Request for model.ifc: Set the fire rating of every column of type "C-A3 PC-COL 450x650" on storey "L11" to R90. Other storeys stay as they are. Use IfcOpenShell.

First a look at what the model holds.

```python
import ifcopenshell
import ifcopenshell.util.element

model = ifcopenshell.open("model.ifc")
print(model.schema)
storey = next(s for s in model.by_type("IfcBuildingStorey") if s.Name == "L11")
columns = [e for e in ifcopenshell.util.element.get_decomposition(storey) if e.is_a("IfcColumn")]
seen = {}
for e in columns:
    element_type = ifcopenshell.util.element.get_type(e)
    key = (element_type.Name if element_type != e and element_type else None, ifcopenshell.util.element.get_pset(e, "Pset_ColumnCommon", "FireRating"))
    seen[key] = seen.get(key, 0) + 1
for (name, value), count in sorted(seen.items(), key=str):
    print(count, "x", name, "|", value)
```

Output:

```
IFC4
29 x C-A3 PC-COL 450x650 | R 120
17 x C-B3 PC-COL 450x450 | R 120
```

```python
import ifcopenshell
import ifcopenshell.api.pset
import ifcopenshell.util.element

model = ifcopenshell.open("model.ifc")

storey = next(s for s in model.by_type("IfcBuildingStorey") if s.Name == "L11")
columns = [e for e in ifcopenshell.util.element.get_decomposition(storey) if e.is_a("IfcColumn")]

count = 0
for e in columns:
    element_type = ifcopenshell.util.element.get_type(e)
    if element_type in (None, e) or element_type.Name != "C-A3 PC-COL 450x650":
        continue
    # add_pset returns the element's existing set when there is one.
    pset = ifcopenshell.api.pset.add_pset(model, product=e, name="Pset_ColumnCommon")
    ifcopenshell.api.pset.edit_pset(model, pset=pset, properties={"FireRating": "R90"})
    count += 1

print(count, "columns updated")

model.write("model_v2.ifc")
```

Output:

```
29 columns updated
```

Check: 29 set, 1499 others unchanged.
